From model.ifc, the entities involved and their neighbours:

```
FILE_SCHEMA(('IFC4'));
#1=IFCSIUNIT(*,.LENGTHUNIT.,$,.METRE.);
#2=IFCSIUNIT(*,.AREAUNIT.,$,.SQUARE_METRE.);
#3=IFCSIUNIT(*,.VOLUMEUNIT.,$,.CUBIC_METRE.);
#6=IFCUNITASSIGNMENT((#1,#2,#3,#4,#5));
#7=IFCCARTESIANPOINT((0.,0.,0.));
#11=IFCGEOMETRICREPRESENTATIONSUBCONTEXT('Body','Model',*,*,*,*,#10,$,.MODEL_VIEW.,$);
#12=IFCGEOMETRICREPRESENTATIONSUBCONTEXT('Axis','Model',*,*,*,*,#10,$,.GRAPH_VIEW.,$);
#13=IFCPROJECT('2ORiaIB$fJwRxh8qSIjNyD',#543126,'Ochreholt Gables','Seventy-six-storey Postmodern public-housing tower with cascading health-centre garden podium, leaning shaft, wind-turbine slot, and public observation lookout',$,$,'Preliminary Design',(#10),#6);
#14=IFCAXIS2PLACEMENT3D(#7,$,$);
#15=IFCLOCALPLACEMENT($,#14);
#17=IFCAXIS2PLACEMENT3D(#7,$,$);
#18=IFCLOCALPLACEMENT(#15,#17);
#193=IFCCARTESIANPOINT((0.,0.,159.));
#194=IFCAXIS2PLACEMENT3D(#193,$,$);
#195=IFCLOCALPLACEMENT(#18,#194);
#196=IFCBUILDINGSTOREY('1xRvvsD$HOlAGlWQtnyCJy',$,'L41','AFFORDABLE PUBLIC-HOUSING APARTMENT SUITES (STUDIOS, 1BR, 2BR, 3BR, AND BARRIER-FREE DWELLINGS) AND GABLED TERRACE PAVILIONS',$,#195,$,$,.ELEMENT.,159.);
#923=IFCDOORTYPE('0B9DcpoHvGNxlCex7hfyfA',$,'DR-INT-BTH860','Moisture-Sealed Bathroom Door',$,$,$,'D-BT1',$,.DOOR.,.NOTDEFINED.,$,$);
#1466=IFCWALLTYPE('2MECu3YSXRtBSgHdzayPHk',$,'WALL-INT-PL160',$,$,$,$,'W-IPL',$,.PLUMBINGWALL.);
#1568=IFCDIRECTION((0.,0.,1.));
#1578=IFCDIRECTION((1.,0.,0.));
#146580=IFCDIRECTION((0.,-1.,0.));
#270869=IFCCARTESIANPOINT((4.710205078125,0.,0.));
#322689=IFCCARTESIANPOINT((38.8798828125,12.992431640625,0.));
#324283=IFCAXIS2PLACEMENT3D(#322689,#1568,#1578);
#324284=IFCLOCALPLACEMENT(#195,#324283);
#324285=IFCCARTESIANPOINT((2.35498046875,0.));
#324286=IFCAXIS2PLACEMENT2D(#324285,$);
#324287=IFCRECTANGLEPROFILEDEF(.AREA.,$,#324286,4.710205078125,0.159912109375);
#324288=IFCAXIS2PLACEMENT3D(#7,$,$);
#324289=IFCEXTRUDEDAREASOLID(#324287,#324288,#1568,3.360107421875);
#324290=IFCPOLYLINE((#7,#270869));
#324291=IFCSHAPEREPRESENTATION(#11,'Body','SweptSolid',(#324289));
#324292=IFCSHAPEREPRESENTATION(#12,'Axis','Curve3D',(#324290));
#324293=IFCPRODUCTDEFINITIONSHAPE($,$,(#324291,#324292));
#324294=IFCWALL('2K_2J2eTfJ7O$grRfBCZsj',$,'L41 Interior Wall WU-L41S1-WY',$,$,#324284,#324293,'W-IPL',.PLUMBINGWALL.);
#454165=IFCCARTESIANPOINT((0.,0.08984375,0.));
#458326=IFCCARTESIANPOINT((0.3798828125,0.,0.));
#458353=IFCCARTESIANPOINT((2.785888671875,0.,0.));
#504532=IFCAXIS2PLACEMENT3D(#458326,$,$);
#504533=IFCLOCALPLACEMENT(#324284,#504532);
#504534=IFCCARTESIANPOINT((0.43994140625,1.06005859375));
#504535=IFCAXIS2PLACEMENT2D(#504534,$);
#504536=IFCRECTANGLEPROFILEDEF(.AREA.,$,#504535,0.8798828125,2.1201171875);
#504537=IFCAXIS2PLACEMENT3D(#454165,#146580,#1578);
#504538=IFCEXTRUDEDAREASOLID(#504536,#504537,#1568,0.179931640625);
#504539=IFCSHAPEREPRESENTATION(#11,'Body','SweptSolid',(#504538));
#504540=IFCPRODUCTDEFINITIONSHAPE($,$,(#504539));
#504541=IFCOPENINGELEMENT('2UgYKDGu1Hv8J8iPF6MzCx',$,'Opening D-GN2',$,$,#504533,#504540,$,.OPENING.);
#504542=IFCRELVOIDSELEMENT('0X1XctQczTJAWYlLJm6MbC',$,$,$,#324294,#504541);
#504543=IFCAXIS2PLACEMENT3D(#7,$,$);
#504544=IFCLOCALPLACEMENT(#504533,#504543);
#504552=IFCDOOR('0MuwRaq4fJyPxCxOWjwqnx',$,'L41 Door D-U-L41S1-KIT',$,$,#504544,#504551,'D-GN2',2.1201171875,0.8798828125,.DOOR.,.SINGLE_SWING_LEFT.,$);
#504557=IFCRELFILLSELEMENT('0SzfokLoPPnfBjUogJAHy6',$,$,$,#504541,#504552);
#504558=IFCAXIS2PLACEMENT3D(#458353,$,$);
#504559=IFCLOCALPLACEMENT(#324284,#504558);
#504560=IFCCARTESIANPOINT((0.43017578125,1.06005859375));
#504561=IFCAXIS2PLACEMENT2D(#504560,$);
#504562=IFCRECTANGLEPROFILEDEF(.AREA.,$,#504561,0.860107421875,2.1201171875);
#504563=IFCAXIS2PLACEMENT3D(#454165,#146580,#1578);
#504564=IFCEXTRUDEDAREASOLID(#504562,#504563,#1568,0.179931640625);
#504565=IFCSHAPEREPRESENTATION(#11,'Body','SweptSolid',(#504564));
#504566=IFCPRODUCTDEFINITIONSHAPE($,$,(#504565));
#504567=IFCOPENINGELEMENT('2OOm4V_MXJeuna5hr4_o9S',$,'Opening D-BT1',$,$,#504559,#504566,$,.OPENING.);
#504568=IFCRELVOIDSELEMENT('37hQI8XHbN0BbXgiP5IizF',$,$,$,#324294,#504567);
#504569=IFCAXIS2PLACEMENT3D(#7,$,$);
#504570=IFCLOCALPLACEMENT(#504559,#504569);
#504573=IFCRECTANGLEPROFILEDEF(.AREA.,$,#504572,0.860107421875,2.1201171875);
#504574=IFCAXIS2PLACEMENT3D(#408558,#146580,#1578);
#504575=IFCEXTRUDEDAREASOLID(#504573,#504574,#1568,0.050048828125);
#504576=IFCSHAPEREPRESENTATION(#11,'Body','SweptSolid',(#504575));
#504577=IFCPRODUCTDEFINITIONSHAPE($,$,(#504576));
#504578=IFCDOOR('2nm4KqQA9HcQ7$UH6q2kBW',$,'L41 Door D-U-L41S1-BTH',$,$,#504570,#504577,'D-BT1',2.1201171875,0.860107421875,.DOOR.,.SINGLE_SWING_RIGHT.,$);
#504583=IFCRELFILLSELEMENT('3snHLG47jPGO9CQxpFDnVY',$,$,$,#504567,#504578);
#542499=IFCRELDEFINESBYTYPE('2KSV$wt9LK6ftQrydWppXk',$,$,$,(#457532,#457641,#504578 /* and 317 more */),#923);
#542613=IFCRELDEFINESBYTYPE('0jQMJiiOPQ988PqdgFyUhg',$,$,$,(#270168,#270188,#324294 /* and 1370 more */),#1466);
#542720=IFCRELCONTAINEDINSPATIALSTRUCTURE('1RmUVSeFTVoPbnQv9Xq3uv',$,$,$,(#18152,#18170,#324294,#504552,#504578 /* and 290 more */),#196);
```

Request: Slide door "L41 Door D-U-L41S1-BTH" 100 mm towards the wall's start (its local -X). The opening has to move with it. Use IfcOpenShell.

```python
import ifcopenshell
import ifcopenshell.api.geometry
import ifcopenshell.util.placement
import ifcopenshell.util.unit

model = ifcopenshell.open("model.ifc")
unit_scale = ifcopenshell.util.unit.calculate_unit_scale(model)

door = model.by_id(504578)
opening = door.FillsVoids[0].RelatingOpeningElement
wall = opening.VoidsElements[0].RelatingBuildingElement

wall_matrix = ifcopenshell.util.placement.get_local_placement(wall.ObjectPlacement)
shift = wall_matrix[:3, 0] * -0.1 / unit_scale
before = ifcopenshell.util.placement.get_local_placement(door.ObjectPlacement)[:3, 3].copy()

# The door is placed relative to its opening, so it follows when the opening moves.
matrix = ifcopenshell.util.placement.get_local_placement(opening.ObjectPlacement)
matrix[:3, 3] += shift
ifcopenshell.api.geometry.edit_object_placement(
    model, product=opening, matrix=matrix, is_si=False, should_transform_children=True
)

after = ifcopenshell.util.placement.get_local_placement(door.ObjectPlacement)[:3, 3]
print("door moved by", (after - before).round(3) + 0.0)

model.write("model_rev.ifc")
```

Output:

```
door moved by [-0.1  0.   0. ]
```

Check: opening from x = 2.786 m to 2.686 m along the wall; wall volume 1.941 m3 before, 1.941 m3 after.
